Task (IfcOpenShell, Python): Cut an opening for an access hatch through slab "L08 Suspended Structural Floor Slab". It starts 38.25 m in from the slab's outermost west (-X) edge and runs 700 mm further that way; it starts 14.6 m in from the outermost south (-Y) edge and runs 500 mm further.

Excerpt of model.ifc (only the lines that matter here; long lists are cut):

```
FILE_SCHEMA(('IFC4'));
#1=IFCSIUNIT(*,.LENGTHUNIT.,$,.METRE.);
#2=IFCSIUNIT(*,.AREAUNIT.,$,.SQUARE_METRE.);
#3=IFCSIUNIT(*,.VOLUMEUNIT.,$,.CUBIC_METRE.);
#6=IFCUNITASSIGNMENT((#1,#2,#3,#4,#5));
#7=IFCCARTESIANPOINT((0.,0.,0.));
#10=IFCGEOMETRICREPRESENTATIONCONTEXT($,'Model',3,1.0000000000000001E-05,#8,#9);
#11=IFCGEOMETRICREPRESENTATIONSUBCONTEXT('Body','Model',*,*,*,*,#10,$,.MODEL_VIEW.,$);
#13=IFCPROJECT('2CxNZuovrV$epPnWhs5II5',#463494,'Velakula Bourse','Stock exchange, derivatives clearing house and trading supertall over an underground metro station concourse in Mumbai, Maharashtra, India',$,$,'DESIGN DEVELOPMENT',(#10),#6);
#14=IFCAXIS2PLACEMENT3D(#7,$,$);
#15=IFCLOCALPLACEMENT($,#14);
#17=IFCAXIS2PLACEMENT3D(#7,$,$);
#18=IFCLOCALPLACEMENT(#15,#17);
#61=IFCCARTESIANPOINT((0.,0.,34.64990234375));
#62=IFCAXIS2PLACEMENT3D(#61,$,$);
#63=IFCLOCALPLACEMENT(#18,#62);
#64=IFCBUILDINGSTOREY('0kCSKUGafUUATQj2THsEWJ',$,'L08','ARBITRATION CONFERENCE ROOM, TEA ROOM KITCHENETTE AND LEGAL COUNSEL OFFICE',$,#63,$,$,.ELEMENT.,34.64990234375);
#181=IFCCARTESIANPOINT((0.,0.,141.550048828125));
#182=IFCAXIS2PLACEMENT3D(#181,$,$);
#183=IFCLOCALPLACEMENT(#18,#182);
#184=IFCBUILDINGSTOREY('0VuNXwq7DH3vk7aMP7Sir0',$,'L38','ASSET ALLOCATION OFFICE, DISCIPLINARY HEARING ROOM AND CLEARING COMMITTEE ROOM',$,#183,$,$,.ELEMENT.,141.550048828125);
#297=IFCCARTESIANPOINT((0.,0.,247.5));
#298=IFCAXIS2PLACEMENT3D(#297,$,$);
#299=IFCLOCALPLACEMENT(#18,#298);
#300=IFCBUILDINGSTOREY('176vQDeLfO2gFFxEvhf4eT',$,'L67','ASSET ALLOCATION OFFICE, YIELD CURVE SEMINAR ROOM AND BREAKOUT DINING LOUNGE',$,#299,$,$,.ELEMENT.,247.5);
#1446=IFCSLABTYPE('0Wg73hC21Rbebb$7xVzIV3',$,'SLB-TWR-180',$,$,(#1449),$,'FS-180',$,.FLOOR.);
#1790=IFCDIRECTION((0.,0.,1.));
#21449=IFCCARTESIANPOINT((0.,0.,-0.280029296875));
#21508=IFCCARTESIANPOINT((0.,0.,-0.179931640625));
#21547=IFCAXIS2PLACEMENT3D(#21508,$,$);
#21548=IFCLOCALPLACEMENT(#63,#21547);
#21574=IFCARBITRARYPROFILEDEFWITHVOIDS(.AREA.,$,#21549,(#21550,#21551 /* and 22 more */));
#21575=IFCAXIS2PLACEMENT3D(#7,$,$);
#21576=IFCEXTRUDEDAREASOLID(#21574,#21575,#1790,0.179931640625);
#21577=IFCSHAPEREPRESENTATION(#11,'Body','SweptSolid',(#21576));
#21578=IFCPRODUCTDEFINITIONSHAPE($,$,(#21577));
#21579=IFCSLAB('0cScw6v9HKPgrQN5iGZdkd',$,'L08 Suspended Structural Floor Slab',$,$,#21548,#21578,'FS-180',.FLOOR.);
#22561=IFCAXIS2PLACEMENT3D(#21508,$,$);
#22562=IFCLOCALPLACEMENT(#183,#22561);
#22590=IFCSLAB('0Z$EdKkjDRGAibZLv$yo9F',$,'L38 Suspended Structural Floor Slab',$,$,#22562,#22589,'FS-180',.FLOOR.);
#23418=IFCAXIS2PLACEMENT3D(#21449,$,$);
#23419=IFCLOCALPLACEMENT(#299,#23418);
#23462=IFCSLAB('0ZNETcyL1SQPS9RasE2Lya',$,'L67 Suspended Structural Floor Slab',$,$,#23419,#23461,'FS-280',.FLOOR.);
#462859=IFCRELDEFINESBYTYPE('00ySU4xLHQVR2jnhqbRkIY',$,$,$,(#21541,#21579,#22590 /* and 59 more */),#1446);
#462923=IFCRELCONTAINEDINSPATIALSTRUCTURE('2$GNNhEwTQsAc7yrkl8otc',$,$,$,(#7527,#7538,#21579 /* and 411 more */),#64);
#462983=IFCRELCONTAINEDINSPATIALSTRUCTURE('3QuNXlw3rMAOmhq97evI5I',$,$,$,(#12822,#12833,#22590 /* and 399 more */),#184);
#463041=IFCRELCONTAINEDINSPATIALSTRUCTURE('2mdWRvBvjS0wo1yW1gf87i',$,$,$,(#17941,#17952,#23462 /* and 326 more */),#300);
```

```python
import numpy as np
import ifcopenshell
import ifcopenshell.api.feature
import ifcopenshell.api.geometry
import ifcopenshell.api.root
import ifcopenshell.geom
import ifcopenshell.util.placement
import ifcopenshell.util.representation
import ifcopenshell.util.shape
import ifcopenshell.util.unit

model = ifcopenshell.open("model.ifc")
unit_scale = ifcopenshell.util.unit.calculate_unit_scale(model)
settings = ifcopenshell.geom.settings()


def volume(element):
    """Net volume in cubic metres, openings subtracted."""
    shape = ifcopenshell.geom.create_shape(settings, element)
    return ifcopenshell.util.shape.get_volume(shape.geometry)


slab = model.by_id(21579)
before = volume(slab)

# Extent in the slab's own axes, in metres. The edges named are its -X and -Y sides.
slab_shape = ifcopenshell.geom.create_shape(settings, slab)
vertices = ifcopenshell.util.shape.get_vertices(slab_shape.geometry)
x_min, y_min, bottom = vertices.min(axis=0)
top = vertices[:, 2].max()

opening = ifcopenshell.api.root.create_entity(model, ifc_class="IfcOpeningElement", name="Access hatch opening", predefined_type="OPENING")
context = ifcopenshell.util.representation.get_context(model, "Model", "Body", "MODEL_VIEW")
width, depth = 0.7, 0.5
outline = [(0.0, 0.0), (width, 0.0), (width, depth), (0.0, depth), (0.0, 0.0)]
# Overshoot both faces by 50 mm so the cut is clean.
shape = ifcopenshell.api.geometry.add_slab_representation(
    model, context=context, depth=top - bottom + 0.1, polyline=outline
)
ifcopenshell.api.geometry.assign_representation(model, product=opening, representation=shape)

matrix = ifcopenshell.util.placement.get_local_placement(slab.ObjectPlacement)
matrix[:, 3] = matrix @ np.append(np.array([x_min + 38.25, y_min + 14.6, bottom - 0.05]) / unit_scale, 1.0)
ifcopenshell.api.geometry.edit_object_placement(model, product=opening, matrix=matrix, is_si=False)
ifcopenshell.api.feature.add_feature(model, feature=opening, element=slab)

after = volume(slab)

print(f"slab volume {before:.3f} -> {after:.3f} m3")

model.write("model_v2.ifc")
```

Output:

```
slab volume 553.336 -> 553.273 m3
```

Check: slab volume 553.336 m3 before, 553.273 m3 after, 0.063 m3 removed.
